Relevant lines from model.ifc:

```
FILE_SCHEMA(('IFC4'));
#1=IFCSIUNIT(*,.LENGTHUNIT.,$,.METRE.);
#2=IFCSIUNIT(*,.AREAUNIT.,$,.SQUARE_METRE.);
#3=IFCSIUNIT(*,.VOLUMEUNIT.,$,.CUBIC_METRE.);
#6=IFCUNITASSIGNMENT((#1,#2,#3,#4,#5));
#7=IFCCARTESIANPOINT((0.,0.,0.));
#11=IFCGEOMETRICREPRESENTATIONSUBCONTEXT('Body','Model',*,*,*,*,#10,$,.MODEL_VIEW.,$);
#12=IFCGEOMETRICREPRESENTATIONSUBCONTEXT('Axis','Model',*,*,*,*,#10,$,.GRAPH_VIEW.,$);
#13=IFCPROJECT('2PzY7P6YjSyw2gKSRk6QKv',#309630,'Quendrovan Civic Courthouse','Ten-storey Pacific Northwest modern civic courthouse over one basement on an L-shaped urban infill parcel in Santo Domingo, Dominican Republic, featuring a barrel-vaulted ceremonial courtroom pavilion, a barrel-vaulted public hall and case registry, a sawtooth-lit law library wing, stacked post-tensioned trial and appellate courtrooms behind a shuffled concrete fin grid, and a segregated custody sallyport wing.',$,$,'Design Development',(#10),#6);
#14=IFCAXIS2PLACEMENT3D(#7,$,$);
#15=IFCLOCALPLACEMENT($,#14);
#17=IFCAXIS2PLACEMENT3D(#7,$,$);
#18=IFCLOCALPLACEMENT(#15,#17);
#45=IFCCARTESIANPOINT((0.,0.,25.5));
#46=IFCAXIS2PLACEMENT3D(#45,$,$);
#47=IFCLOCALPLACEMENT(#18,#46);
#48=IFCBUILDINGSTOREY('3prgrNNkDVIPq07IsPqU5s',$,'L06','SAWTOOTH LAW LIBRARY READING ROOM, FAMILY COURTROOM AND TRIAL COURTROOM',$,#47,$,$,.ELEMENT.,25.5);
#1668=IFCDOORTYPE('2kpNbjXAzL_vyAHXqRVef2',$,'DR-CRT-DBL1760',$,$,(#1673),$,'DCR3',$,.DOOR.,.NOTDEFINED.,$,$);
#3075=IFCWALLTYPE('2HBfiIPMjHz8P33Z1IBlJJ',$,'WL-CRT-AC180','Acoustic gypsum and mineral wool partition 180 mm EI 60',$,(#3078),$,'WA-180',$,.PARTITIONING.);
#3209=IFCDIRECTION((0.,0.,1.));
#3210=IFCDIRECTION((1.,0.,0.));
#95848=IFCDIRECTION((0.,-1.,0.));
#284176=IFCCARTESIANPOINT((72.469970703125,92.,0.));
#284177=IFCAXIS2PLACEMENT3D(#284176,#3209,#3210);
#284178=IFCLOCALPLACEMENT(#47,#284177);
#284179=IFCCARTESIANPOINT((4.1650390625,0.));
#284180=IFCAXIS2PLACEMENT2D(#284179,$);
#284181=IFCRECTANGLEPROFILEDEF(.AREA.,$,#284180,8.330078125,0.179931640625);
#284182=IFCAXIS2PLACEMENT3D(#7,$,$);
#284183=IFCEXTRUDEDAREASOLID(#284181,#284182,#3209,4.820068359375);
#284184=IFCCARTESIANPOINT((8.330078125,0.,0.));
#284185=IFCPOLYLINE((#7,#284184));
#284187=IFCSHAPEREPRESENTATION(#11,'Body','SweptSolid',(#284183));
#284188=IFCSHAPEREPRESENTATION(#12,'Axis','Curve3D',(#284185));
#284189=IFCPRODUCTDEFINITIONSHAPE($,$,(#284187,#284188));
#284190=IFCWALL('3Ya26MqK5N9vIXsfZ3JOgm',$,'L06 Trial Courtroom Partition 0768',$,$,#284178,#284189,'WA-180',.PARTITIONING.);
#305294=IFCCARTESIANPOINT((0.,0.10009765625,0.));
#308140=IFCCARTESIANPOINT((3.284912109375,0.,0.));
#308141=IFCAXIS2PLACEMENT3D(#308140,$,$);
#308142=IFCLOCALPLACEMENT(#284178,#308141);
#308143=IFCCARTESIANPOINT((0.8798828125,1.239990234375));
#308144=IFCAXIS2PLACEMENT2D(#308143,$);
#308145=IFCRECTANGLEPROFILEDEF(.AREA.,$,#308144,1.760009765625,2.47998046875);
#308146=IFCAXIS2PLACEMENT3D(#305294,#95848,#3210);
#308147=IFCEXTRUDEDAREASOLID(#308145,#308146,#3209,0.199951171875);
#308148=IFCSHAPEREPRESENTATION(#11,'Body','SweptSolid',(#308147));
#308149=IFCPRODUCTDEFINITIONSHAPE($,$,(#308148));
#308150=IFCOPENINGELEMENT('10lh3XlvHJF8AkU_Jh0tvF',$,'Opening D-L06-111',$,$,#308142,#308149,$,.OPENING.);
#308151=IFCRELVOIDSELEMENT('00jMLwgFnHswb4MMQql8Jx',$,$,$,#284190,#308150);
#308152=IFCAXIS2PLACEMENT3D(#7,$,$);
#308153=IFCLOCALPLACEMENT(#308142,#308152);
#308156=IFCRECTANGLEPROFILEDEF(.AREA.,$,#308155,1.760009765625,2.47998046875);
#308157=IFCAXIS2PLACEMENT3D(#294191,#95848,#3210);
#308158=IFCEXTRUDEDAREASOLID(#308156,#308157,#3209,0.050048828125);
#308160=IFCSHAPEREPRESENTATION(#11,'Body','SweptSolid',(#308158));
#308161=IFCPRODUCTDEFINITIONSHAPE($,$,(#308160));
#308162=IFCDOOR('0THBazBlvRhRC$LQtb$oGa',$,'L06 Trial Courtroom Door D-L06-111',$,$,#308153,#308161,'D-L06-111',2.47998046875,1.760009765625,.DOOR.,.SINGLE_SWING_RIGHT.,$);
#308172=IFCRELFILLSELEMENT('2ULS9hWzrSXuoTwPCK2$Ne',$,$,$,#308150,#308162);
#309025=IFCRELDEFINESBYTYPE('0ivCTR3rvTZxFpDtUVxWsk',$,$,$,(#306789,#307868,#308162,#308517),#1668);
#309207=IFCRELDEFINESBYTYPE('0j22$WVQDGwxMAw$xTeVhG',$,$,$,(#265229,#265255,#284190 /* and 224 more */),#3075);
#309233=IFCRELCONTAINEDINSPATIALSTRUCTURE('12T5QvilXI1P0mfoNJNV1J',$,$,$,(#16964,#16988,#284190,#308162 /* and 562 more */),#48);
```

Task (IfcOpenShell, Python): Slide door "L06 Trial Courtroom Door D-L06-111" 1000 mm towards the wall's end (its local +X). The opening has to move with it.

```python
import ifcopenshell
import ifcopenshell.api.geometry
import ifcopenshell.util.placement
import ifcopenshell.util.unit

model = ifcopenshell.open("model.ifc")
unit_scale = ifcopenshell.util.unit.calculate_unit_scale(model)

door = model.by_guid("0THBazBlvRhRC$LQtb$oGa")
opening = door.FillsVoids[0].RelatingOpeningElement
wall = opening.VoidsElements[0].RelatingBuildingElement

wall_matrix = ifcopenshell.util.placement.get_local_placement(wall.ObjectPlacement)
shift = wall_matrix[:3, 0] * 1 / unit_scale
before = ifcopenshell.util.placement.get_local_placement(door.ObjectPlacement)[:3, 3].copy()

# The door is placed relative to its opening, so it follows when the opening moves.
matrix = ifcopenshell.util.placement.get_local_placement(opening.ObjectPlacement)
matrix[:3, 3] += shift
ifcopenshell.api.geometry.edit_object_placement(
    model, product=opening, matrix=matrix, is_si=False, should_transform_children=True
)

after = ifcopenshell.util.placement.get_local_placement(door.ObjectPlacement)[:3, 3]
print("door moved by", (after - before).round(3) + 0.0)

model.write("model_updated.ifc")
```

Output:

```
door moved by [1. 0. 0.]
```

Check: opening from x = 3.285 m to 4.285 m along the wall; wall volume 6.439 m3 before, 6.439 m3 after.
